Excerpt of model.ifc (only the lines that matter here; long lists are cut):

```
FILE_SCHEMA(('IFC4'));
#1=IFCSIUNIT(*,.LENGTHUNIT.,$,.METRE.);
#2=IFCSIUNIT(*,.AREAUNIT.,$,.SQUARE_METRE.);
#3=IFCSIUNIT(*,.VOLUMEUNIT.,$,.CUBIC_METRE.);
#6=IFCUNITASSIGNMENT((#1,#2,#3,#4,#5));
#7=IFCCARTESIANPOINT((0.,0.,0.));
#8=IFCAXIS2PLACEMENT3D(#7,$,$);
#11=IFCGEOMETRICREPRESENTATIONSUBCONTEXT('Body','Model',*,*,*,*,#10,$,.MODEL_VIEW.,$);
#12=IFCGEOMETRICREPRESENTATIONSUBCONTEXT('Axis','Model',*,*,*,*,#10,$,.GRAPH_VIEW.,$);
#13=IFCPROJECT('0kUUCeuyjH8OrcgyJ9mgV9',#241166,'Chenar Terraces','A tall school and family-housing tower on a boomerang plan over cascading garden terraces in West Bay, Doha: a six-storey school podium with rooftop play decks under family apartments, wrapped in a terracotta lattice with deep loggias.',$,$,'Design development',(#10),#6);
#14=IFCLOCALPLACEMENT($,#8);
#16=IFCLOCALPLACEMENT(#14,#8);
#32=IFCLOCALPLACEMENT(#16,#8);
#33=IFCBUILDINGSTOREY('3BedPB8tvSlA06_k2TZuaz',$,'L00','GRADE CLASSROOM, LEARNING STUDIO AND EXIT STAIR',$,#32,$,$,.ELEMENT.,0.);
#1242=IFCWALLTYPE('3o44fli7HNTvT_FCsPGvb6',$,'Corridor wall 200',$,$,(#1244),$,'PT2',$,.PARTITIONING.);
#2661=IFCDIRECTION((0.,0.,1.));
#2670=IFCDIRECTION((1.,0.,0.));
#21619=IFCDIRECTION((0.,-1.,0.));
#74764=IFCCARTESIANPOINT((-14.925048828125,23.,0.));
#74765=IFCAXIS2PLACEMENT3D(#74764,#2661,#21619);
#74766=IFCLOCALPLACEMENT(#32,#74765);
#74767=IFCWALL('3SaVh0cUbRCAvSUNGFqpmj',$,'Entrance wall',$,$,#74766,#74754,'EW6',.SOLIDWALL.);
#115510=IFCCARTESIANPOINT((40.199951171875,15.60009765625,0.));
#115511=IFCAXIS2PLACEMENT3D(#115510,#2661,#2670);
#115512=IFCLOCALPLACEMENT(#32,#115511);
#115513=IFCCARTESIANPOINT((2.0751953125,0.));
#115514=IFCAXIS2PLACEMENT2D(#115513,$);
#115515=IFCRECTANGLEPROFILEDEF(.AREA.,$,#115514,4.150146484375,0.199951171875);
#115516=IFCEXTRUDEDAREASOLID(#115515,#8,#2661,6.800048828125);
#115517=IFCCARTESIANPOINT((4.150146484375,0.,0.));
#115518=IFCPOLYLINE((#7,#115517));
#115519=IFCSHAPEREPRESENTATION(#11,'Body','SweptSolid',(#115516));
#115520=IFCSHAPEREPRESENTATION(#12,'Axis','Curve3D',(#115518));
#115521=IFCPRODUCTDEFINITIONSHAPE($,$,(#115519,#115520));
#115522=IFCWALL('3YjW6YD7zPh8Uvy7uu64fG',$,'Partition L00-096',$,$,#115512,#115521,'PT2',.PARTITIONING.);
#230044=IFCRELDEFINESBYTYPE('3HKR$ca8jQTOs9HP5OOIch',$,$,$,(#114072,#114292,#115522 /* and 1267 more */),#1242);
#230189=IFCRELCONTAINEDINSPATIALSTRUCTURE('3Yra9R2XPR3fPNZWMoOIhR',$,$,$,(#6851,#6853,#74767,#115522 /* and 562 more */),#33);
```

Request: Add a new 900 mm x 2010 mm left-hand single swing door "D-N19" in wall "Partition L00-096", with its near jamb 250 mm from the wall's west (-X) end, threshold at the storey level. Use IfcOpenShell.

```python
import numpy as np
import ifcopenshell
import ifcopenshell.api.feature
import ifcopenshell.api.geometry
import ifcopenshell.api.root
import ifcopenshell.api.spatial
import ifcopenshell.geom
import ifcopenshell.util.element
import ifcopenshell.util.placement
import ifcopenshell.util.representation
import ifcopenshell.util.shape
import ifcopenshell.util.unit

model = ifcopenshell.open("model.ifc")
unit_scale = ifcopenshell.util.unit.calculate_unit_scale(model)
settings = ifcopenshell.geom.settings()


def volume(element):
    """Net volume in cubic metres, openings subtracted."""
    shape = ifcopenshell.geom.create_shape(settings, element)
    return ifcopenshell.util.shape.get_volume(shape.geometry)


wall = model.by_guid("3YjW6YD7zPh8Uvy7uu64fG")
storey = ifcopenshell.util.element.get_container(wall, ifc_class="IfcBuildingStorey")
context = ifcopenshell.util.representation.get_context(model, "Model", "Body", "MODEL_VIEW")
before = volume(wall)

width, height, from_end, sill = 0.9, 2.01, 0.25, 0.0  # metres

# The wall runs along its own X axis, and the end named is its -X end.
wall_shape = ifcopenshell.geom.create_shape(settings, wall)
x, y, z = ifcopenshell.util.shape.get_vertices(wall_shape.geometry).T
start = x.min() + from_end
face, thickness = float(y.min()), float(y.max() - y.min())
wall_matrix = ifcopenshell.util.placement.get_local_placement(wall.ObjectPlacement)
level = ifcopenshell.util.placement.get_local_placement(storey.ObjectPlacement)[2, 3]


def in_wall(x, y):
    """Placement at x, y metres in the wall's axes, at sill height."""
    matrix = wall_matrix.copy()
    matrix[:, 3] = wall_matrix @ np.array([x / unit_scale, y / unit_scale, 0.0, 1.0])
    matrix[2, 3] = level + sill / unit_scale
    return matrix


# Opening: a box that overshoots both wall faces by 50 mm.
opening = ifcopenshell.api.root.create_entity(model, ifc_class="IfcOpeningElement", predefined_type="OPENING")
box = ifcopenshell.api.geometry.add_wall_representation(
    model, context=context, length=width, height=height, thickness=thickness + 0.1
)
ifcopenshell.api.geometry.assign_representation(model, product=opening, representation=box)
ifcopenshell.api.geometry.edit_object_placement(model, product=opening, matrix=in_wall(start, face - 0.05), is_si=False)
ifcopenshell.api.feature.add_feature(model, feature=opening, element=wall)

door = ifcopenshell.api.root.create_entity(model, ifc_class="IfcDoor", name="D-N19", predefined_type="DOOR")
door.OverallWidth, door.OverallHeight = width / unit_scale, height / unit_scale
door.OperationType = "SINGLE_SWING_LEFT"
body = ifcopenshell.api.geometry.add_door_representation(
    model,
    context=context,
    overall_width=door.OverallWidth,
    overall_height=door.OverallHeight,
    operation_type="SINGLE_SWING_LEFT",
    lining_properties={"LiningDepth": thickness / unit_scale, "ThresholdDepth": thickness / unit_scale},
)
ifcopenshell.api.geometry.assign_representation(model, product=door, representation=body)
ifcopenshell.api.spatial.assign_container(model, products=[door], relating_structure=storey)
ifcopenshell.api.feature.add_filling(model, opening=opening, element=door)

# The lining spans the wall, so the door starts at the wall face.
ifcopenshell.api.geometry.edit_object_placement(model, product=door, matrix=in_wall(start, face), is_si=False)

after = volume(wall)

print(f"wall volume {before:.3f} -> {after:.3f} m3")

model.write("model-out.ifc")
```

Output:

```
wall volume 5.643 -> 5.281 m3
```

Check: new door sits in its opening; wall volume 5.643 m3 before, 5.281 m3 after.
